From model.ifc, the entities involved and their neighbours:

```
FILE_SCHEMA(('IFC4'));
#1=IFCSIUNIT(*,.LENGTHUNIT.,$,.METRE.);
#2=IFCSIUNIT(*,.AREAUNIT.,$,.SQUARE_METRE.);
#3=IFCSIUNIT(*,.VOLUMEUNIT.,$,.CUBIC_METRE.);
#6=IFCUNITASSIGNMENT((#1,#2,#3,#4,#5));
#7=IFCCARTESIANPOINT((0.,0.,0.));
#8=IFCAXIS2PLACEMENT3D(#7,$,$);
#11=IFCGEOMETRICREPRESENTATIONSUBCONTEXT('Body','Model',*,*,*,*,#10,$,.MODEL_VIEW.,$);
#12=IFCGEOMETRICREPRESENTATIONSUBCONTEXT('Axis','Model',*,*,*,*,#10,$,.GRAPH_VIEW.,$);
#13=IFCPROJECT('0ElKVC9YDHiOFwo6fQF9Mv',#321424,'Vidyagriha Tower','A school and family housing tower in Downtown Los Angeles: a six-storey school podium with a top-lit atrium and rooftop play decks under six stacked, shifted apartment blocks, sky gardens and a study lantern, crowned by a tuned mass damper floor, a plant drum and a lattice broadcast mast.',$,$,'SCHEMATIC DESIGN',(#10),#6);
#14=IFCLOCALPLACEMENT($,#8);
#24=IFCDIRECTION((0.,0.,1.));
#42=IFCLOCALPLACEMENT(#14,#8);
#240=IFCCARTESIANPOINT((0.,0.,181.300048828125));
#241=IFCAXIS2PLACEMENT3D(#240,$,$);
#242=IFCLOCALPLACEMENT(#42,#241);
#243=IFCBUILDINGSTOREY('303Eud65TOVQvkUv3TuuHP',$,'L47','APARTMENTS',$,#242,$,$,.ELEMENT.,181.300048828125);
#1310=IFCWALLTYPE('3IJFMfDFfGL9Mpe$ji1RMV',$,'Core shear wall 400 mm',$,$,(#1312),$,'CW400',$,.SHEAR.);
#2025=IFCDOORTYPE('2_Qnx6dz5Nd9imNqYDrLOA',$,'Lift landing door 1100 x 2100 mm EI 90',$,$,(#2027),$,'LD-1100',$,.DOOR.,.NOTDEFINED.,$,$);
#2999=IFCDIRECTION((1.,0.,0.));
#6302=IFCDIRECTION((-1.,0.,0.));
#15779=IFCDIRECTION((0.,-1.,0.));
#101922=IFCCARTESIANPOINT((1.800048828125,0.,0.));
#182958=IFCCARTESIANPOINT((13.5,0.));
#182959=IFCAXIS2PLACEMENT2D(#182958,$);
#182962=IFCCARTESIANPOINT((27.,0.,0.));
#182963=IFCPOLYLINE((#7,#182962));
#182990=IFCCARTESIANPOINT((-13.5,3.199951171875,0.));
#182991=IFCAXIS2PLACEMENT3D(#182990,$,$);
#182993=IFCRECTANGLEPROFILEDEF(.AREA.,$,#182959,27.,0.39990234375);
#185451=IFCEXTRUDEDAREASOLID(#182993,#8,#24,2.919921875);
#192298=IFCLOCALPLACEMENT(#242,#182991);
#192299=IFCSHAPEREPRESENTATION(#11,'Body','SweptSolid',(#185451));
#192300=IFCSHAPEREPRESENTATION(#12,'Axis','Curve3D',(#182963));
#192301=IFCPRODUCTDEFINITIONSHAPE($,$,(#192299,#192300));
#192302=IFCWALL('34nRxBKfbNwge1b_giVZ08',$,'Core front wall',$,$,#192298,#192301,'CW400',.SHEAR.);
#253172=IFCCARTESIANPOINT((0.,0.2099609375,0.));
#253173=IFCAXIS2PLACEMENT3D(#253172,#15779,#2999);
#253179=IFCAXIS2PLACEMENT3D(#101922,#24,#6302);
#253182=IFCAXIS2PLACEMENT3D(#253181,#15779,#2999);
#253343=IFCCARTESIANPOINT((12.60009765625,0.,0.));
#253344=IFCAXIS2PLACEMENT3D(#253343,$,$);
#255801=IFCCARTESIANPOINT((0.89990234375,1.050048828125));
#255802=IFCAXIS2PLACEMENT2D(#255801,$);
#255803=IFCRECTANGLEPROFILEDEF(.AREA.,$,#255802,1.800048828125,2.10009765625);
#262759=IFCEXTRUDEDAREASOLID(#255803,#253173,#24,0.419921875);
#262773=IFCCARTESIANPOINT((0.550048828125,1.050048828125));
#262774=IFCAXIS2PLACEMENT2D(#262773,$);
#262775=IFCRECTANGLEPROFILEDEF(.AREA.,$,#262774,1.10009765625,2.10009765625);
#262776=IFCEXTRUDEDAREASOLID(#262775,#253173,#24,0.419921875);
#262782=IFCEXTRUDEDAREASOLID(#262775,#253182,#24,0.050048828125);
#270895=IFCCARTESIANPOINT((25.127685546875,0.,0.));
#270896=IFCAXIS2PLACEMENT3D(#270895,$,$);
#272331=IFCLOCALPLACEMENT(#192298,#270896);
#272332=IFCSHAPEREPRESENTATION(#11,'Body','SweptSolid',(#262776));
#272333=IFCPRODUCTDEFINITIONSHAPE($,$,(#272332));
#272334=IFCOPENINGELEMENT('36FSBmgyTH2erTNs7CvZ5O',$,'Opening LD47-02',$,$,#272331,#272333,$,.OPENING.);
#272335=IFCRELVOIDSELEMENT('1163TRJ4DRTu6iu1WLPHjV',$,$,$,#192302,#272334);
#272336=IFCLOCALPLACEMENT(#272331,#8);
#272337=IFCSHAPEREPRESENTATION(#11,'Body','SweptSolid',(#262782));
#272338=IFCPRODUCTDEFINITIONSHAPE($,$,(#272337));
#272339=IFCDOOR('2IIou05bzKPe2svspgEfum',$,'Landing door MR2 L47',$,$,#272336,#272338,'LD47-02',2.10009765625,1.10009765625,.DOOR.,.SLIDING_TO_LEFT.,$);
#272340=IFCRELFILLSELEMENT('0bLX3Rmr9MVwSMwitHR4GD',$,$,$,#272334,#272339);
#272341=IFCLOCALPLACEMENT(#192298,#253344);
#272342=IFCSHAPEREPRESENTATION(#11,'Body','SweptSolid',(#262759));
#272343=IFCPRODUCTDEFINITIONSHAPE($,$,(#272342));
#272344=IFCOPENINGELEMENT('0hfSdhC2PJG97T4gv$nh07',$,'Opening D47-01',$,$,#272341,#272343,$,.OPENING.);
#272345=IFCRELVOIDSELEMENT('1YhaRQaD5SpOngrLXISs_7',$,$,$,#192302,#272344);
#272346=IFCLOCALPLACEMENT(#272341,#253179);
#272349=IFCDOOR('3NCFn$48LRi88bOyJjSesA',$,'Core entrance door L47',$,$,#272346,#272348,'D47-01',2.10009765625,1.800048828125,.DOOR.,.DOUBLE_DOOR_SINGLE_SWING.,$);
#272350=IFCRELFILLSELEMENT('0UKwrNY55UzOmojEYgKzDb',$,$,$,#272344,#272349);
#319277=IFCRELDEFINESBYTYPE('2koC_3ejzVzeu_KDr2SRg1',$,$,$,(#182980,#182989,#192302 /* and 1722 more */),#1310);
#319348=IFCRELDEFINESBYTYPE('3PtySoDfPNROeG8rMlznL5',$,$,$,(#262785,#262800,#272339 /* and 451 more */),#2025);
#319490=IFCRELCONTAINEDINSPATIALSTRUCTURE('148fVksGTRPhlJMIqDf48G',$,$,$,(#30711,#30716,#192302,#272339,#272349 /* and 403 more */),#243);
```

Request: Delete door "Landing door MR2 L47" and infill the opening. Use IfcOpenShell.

```python
import ifcopenshell
import ifcopenshell.api.feature
import ifcopenshell.api.root
import ifcopenshell.geom
import ifcopenshell.util.shape

model = ifcopenshell.open("model.ifc")
settings = ifcopenshell.geom.settings()


def volume(element):
    """Net volume in cubic metres, openings subtracted."""
    shape = ifcopenshell.geom.create_shape(settings, element)
    return ifcopenshell.util.shape.get_volume(shape.geometry)


door = model.by_id(272339)
opening = door.FillsVoids[0].RelatingOpeningElement
wall = opening.VoidsElements[0].RelatingBuildingElement
before = volume(wall)

ifcopenshell.api.root.remove_product(model, product=door)
ifcopenshell.api.feature.remove_feature(model, feature=opening)

after = volume(wall)

print(f"wall volume {before:.3f} -> {after:.3f} m3")

model.write("model-out.ifc")
```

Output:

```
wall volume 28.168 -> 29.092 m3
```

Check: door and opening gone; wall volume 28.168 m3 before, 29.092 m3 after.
